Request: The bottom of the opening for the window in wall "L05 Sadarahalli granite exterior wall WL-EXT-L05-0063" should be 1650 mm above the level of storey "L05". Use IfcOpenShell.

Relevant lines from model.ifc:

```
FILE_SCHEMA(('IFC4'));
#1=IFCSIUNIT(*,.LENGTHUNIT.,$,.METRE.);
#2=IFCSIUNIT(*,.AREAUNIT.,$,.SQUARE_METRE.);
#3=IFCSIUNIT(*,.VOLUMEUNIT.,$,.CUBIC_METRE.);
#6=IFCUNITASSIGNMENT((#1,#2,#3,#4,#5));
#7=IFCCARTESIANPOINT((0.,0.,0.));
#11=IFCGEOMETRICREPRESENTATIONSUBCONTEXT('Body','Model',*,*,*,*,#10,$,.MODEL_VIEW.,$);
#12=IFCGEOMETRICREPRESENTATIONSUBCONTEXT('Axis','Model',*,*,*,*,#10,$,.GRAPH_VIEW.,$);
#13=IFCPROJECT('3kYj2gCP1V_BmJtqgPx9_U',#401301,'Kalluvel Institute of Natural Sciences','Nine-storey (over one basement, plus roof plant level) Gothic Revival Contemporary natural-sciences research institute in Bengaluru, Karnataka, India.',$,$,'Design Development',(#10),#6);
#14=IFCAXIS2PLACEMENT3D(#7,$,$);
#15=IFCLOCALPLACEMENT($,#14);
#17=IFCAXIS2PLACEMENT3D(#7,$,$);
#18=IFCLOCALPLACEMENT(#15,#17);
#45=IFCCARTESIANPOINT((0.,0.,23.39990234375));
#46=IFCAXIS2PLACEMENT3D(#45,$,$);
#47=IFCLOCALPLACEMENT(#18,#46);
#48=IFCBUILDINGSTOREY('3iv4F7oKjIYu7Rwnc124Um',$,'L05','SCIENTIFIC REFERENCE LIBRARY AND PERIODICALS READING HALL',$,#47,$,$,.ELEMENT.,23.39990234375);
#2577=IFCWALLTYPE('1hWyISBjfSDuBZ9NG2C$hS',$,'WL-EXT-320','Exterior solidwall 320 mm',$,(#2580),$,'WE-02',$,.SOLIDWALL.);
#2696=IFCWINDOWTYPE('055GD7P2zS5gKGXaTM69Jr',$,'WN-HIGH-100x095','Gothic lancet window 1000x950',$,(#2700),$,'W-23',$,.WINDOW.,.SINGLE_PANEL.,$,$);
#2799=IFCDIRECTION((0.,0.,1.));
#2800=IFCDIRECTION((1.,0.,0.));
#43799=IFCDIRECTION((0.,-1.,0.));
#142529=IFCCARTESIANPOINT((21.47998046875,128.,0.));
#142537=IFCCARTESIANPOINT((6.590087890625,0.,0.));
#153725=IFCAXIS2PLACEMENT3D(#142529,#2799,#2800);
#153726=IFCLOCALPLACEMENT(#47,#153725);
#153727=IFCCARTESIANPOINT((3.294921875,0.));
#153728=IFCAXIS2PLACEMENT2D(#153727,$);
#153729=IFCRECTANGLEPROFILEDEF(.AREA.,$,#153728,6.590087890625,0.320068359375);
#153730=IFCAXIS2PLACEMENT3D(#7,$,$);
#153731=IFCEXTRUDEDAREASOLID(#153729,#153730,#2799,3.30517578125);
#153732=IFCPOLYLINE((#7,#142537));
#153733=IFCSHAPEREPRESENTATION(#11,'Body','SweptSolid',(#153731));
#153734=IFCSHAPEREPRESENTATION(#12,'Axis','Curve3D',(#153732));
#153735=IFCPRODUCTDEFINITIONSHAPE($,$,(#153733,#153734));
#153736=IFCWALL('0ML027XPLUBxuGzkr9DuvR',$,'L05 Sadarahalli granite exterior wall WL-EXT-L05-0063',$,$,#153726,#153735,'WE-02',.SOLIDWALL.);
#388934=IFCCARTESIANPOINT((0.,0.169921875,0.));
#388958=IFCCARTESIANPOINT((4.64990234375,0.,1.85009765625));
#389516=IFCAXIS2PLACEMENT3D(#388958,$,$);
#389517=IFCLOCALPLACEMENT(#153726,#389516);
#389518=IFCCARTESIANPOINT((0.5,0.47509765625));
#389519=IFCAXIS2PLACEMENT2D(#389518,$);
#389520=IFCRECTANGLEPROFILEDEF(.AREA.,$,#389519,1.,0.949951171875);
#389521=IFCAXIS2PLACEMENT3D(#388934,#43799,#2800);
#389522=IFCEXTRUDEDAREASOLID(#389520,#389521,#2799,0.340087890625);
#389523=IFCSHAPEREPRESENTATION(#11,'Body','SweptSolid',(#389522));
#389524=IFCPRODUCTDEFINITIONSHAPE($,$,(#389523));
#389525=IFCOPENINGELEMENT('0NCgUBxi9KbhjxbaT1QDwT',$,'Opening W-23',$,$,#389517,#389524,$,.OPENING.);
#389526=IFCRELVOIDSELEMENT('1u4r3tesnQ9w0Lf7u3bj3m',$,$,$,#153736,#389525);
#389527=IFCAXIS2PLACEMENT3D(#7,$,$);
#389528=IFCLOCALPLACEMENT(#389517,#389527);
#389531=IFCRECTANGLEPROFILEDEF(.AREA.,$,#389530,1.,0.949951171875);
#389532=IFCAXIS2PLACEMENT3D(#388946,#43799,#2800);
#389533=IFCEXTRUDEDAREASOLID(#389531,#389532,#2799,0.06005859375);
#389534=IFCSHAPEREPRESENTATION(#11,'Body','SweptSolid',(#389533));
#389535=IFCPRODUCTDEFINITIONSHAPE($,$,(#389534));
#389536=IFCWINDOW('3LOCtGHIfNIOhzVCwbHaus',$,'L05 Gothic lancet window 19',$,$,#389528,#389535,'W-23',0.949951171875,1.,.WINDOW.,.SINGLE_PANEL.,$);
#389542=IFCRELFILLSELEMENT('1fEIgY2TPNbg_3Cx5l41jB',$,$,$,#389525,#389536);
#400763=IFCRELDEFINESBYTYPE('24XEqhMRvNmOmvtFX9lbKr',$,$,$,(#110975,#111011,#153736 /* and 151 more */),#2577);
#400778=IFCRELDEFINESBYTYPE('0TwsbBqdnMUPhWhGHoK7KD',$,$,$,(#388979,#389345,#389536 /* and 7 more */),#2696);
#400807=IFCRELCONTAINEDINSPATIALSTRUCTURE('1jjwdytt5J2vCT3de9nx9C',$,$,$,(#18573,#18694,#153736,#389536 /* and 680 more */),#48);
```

```python
import numpy as np
import ifcopenshell
import ifcopenshell.api.geometry
import ifcopenshell.geom
import ifcopenshell.util.element
import ifcopenshell.util.placement
import ifcopenshell.util.shape
import ifcopenshell.util.unit

model = ifcopenshell.open("model.ifc")
unit_scale = ifcopenshell.util.unit.calculate_unit_scale(model)

window = model.by_guid("3LOCtGHIfNIOhzVCwbHaus")
opening = window.FillsVoids[0].RelatingOpeningElement
storey = ifcopenshell.util.element.get_container(window, ifc_class="IfcBuildingStorey")
level = ifcopenshell.util.placement.get_local_placement(storey.ObjectPlacement)[2, 3]

# The opening's origin need not be at the sill, so measure its lowest point.
shape = ifcopenshell.geom.create_shape(ifcopenshell.geom.settings(), opening)
bottom = ifcopenshell.util.shape.get_shape_bottom_elevation(shape, shape.geometry) / unit_scale
dz = level + 1.65 / unit_scale - bottom

shift = np.array([0.0, 0.0, dz])
# The window is placed relative to its opening, so it follows when the opening moves.
matrix = ifcopenshell.util.placement.get_local_placement(opening.ObjectPlacement)
matrix[:3, 3] += shift
ifcopenshell.api.geometry.edit_object_placement(
    model, product=opening, matrix=matrix, is_si=False, should_transform_children=True
)

print(f"moved by {dz * unit_scale:+.3f} m")

model.write("model_updated.ifc")
```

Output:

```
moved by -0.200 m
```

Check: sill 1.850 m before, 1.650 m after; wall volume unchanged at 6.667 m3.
